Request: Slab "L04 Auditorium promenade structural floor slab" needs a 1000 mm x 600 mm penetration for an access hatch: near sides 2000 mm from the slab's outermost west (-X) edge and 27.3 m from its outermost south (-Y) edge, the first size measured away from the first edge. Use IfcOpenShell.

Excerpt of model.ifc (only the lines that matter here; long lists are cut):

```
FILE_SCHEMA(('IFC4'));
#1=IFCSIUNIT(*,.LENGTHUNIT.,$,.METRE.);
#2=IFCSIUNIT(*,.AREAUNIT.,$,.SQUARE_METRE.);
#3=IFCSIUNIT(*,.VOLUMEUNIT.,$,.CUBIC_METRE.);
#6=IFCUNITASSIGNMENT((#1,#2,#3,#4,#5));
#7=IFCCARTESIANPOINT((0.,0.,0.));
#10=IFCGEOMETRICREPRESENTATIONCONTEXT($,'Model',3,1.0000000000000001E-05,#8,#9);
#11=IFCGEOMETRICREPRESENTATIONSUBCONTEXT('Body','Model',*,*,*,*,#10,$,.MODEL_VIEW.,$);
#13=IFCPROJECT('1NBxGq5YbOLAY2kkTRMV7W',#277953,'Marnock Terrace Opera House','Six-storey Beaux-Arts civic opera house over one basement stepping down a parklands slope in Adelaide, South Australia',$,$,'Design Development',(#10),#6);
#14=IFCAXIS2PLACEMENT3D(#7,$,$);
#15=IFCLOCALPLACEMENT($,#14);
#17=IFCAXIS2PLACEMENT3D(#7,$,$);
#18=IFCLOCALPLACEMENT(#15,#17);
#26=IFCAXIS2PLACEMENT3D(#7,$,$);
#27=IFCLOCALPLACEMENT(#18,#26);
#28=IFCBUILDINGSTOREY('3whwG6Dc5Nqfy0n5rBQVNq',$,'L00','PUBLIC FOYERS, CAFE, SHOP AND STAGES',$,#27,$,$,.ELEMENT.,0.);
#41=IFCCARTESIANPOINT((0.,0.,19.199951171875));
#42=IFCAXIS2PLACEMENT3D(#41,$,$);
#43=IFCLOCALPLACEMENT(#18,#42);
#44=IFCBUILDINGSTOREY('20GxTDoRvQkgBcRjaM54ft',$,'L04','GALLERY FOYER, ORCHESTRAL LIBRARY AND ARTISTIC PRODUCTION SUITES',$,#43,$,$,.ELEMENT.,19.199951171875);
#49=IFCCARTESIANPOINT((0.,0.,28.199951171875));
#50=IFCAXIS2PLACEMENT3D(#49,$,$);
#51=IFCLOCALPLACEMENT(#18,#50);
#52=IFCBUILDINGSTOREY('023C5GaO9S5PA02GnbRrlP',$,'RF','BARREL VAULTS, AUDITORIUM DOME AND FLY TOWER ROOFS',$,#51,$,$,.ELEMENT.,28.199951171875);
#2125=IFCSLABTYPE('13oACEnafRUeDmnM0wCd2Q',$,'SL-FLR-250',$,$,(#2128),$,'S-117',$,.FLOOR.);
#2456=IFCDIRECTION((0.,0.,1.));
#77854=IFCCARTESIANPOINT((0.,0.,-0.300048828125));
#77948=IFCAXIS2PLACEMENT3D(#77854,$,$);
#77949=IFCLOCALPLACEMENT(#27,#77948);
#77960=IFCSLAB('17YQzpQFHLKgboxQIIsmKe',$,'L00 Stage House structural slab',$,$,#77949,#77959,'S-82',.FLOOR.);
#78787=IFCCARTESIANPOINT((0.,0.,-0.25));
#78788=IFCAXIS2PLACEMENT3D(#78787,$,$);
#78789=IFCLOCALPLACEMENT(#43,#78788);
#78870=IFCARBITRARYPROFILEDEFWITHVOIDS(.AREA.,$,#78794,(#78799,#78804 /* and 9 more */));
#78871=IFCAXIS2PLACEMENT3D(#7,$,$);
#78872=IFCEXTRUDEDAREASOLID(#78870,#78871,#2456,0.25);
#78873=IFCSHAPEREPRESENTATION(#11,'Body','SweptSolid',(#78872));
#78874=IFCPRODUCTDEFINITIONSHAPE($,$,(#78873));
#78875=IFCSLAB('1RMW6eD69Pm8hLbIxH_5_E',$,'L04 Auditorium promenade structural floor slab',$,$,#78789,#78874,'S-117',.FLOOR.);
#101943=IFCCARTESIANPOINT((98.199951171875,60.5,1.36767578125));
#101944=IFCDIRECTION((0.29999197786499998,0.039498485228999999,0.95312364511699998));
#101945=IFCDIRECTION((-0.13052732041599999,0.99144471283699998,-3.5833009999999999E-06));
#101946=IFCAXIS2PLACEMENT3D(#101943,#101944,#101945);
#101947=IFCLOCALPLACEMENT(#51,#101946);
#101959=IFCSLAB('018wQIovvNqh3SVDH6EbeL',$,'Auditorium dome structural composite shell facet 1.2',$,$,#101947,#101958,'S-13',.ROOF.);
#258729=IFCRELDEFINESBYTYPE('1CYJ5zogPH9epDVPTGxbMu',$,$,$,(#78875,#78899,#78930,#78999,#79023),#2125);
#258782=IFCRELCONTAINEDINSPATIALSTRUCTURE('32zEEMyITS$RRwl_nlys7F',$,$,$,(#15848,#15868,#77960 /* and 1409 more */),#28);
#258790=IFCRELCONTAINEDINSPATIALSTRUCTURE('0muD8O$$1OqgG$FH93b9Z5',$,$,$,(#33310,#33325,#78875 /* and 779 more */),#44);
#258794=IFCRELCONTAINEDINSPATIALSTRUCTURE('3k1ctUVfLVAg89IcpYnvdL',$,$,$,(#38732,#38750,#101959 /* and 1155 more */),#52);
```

```python
import numpy as np
import ifcopenshell
import ifcopenshell.api.feature
import ifcopenshell.api.geometry
import ifcopenshell.api.root
import ifcopenshell.geom
import ifcopenshell.util.placement
import ifcopenshell.util.representation
import ifcopenshell.util.shape
import ifcopenshell.util.unit

model = ifcopenshell.open("model.ifc")
unit_scale = ifcopenshell.util.unit.calculate_unit_scale(model)
settings = ifcopenshell.geom.settings()


def volume(element):
    """Net volume in cubic metres, openings subtracted."""
    shape = ifcopenshell.geom.create_shape(settings, element)
    return ifcopenshell.util.shape.get_volume(shape.geometry)


slab = model.by_guid("1RMW6eD69Pm8hLbIxH_5_E")
before = volume(slab)

# Extent in the slab's own axes, in metres. The edges named are its -X and -Y sides.
slab_shape = ifcopenshell.geom.create_shape(settings, slab)
vertices = ifcopenshell.util.shape.get_vertices(slab_shape.geometry)
x_min, y_min, bottom = vertices.min(axis=0)
top = vertices[:, 2].max()

opening = ifcopenshell.api.root.create_entity(model, ifc_class="IfcOpeningElement", name="Access hatch opening", predefined_type="OPENING")
context = ifcopenshell.util.representation.get_context(model, "Model", "Body", "MODEL_VIEW")
width, depth = 1, 0.6
outline = [(0.0, 0.0), (width, 0.0), (width, depth), (0.0, depth), (0.0, 0.0)]
# Overshoot both faces by 50 mm so the cut is clean.
shape = ifcopenshell.api.geometry.add_slab_representation(
    model, context=context, depth=top - bottom + 0.1, polyline=outline
)
ifcopenshell.api.geometry.assign_representation(model, product=opening, representation=shape)

matrix = ifcopenshell.util.placement.get_local_placement(slab.ObjectPlacement)
matrix[:, 3] = matrix @ np.append(np.array([x_min + 2, y_min + 27.3, bottom - 0.05]) / unit_scale, 1.0)
ifcopenshell.api.geometry.edit_object_placement(model, product=opening, matrix=matrix, is_si=False)
ifcopenshell.api.feature.add_feature(model, feature=opening, element=slab)

after = volume(slab)

print(f"slab volume {before:.3f} -> {after:.3f} m3")

model.write("model_v2.ifc")
```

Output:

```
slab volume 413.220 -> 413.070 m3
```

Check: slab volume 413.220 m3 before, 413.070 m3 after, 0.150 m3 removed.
